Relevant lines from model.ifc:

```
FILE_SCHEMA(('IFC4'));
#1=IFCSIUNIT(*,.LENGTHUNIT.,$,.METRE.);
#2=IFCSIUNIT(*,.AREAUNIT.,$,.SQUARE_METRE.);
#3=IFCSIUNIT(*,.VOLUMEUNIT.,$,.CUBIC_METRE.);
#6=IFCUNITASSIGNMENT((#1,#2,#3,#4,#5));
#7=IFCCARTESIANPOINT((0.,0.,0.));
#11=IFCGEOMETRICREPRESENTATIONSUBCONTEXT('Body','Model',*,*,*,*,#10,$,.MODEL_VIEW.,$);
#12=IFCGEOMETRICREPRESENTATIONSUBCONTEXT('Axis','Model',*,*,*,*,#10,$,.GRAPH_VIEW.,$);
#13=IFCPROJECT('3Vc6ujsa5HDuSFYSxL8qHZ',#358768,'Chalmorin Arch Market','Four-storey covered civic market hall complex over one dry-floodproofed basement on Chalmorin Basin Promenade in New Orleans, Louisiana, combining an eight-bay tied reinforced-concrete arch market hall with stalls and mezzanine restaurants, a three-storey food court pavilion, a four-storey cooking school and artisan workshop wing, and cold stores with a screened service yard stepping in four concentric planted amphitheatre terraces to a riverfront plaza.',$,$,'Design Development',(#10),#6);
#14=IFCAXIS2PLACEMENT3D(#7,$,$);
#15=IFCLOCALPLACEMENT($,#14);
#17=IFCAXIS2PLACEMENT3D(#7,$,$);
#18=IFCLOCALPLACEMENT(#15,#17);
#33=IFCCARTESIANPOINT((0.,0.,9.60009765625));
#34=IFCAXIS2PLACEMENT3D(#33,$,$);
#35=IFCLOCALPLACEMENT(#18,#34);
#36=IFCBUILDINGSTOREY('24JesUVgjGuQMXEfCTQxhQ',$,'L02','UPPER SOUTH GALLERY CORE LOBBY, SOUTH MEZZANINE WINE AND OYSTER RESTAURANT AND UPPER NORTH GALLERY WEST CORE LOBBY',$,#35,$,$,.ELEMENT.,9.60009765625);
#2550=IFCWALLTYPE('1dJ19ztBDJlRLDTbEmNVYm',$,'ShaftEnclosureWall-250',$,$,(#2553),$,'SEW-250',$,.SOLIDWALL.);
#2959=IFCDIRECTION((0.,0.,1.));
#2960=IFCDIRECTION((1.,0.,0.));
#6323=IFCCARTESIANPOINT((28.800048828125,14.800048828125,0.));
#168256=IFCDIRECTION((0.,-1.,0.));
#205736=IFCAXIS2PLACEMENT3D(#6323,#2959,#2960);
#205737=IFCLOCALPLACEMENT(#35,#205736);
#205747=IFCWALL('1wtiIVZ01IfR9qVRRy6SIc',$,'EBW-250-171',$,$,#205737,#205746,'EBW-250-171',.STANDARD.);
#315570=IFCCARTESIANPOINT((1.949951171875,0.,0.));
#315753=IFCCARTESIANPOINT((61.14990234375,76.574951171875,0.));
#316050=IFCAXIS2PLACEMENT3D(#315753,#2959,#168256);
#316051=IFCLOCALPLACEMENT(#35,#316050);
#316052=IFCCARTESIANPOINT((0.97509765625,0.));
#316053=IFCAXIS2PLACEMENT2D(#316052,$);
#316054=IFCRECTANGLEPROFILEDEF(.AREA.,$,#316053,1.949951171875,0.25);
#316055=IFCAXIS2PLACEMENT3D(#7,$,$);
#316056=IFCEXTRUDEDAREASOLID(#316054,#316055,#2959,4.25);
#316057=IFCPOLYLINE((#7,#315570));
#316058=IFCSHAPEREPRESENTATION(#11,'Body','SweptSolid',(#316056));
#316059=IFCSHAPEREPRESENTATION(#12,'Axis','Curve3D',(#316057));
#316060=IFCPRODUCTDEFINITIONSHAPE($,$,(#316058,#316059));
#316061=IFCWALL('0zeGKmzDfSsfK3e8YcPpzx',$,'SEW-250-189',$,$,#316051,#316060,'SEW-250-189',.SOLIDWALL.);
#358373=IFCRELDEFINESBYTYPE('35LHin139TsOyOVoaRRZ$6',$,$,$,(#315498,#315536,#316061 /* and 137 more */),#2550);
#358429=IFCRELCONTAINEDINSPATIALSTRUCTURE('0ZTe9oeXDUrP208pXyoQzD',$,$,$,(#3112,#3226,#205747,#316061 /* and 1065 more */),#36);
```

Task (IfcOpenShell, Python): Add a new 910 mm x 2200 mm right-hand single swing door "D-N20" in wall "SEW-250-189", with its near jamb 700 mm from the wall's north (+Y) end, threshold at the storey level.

```python
import numpy as np
import ifcopenshell
import ifcopenshell.api.feature
import ifcopenshell.api.geometry
import ifcopenshell.api.root
import ifcopenshell.api.spatial
import ifcopenshell.geom
import ifcopenshell.util.element
import ifcopenshell.util.placement
import ifcopenshell.util.representation
import ifcopenshell.util.shape
import ifcopenshell.util.unit

model = ifcopenshell.open("model.ifc")
unit_scale = ifcopenshell.util.unit.calculate_unit_scale(model)
settings = ifcopenshell.geom.settings()


def volume(element):
    """Net volume in cubic metres, openings subtracted."""
    shape = ifcopenshell.geom.create_shape(settings, element)
    return ifcopenshell.util.shape.get_volume(shape.geometry)


wall = model.by_guid("0zeGKmzDfSsfK3e8YcPpzx")
storey = ifcopenshell.util.element.get_container(wall, ifc_class="IfcBuildingStorey")
context = ifcopenshell.util.representation.get_context(model, "Model", "Body", "MODEL_VIEW")
before = volume(wall)

width, height, from_end, sill = 0.91, 2.2, 0.7, 0.0  # metres

# The wall runs along its own X axis, and the end named is its -X end.
wall_shape = ifcopenshell.geom.create_shape(settings, wall)
x, y, z = ifcopenshell.util.shape.get_vertices(wall_shape.geometry).T
start = x.min() + from_end
face, thickness = float(y.min()), float(y.max() - y.min())
wall_matrix = ifcopenshell.util.placement.get_local_placement(wall.ObjectPlacement)
level = ifcopenshell.util.placement.get_local_placement(storey.ObjectPlacement)[2, 3]


def in_wall(x, y):
    """Placement at x, y metres in the wall's axes, at sill height."""
    matrix = wall_matrix.copy()
    matrix[:, 3] = wall_matrix @ np.array([x / unit_scale, y / unit_scale, 0.0, 1.0])
    matrix[2, 3] = level + sill / unit_scale
    return matrix


# Opening: a box that overshoots both wall faces by 50 mm.
opening = ifcopenshell.api.root.create_entity(model, ifc_class="IfcOpeningElement", predefined_type="OPENING")
box = ifcopenshell.api.geometry.add_wall_representation(
    model, context=context, length=width, height=height, thickness=thickness + 0.1
)
ifcopenshell.api.geometry.assign_representation(model, product=opening, representation=box)
ifcopenshell.api.geometry.edit_object_placement(model, product=opening, matrix=in_wall(start, face - 0.05), is_si=False)
ifcopenshell.api.feature.add_feature(model, feature=opening, element=wall)

door = ifcopenshell.api.root.create_entity(model, ifc_class="IfcDoor", name="D-N20", predefined_type="DOOR")
door.OverallWidth, door.OverallHeight = width / unit_scale, height / unit_scale
door.OperationType = "SINGLE_SWING_RIGHT"
body = ifcopenshell.api.geometry.add_door_representation(
    model,
    context=context,
    overall_width=door.OverallWidth,
    overall_height=door.OverallHeight,
    operation_type="SINGLE_SWING_RIGHT",
    lining_properties={"LiningDepth": thickness / unit_scale, "ThresholdDepth": thickness / unit_scale},
)
ifcopenshell.api.geometry.assign_representation(model, product=door, representation=body)
ifcopenshell.api.spatial.assign_container(model, products=[door], relating_structure=storey)
ifcopenshell.api.feature.add_filling(model, opening=opening, element=door)

# The lining spans the wall, so the door starts at the wall face.
ifcopenshell.api.geometry.edit_object_placement(model, product=door, matrix=in_wall(start, face), is_si=False)

after = volume(wall)

print(f"wall volume {before:.3f} -> {after:.3f} m3")

model.write("model_edited.ifc")
```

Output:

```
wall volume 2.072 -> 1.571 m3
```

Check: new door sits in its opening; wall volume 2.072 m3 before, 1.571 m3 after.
